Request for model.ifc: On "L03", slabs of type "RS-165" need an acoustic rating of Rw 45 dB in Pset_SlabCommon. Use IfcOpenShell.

First a look at what the model holds.

```python
import ifcopenshell
import ifcopenshell.util.element

model = ifcopenshell.open("model.ifc")
print(model.schema)
storey = next(s for s in model.by_type("IfcBuildingStorey") if s.Name == "L03")
slabs = [e for e in ifcopenshell.util.element.get_decomposition(storey) if e.is_a("IfcSlab")]
seen = {}
for e in slabs:
    element_type = ifcopenshell.util.element.get_type(e)
    key = (element_type.Name if element_type != e and element_type else None, ifcopenshell.util.element.get_pset(e, "Pset_SlabCommon", "AcousticRating"))
    seen[key] = seen.get(key, 0) + 1
for (name, value), count in sorted(seen.items(), key=str):
    print(count, "x", name, "|", value)
```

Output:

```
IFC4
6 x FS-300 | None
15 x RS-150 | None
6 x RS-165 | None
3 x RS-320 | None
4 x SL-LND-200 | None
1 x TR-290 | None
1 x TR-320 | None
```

```python
import ifcopenshell
import ifcopenshell.api.pset
import ifcopenshell.util.element

model = ifcopenshell.open("model.ifc")

storey = next(s for s in model.by_type("IfcBuildingStorey") if s.Name == "L03")
slabs = [e for e in ifcopenshell.util.element.get_decomposition(storey) if e.is_a("IfcSlab")]

count = 0
for e in slabs:
    element_type = ifcopenshell.util.element.get_type(e)
    if element_type in (None, e) or element_type.Name != "RS-165":
        continue
    # add_pset returns the element's existing set when there is one.
    pset = ifcopenshell.api.pset.add_pset(model, product=e, name="Pset_SlabCommon")
    ifcopenshell.api.pset.edit_pset(model, pset=pset, properties={"AcousticRating": "Rw 45 dB"})
    count += 1

print(count, "slabs updated")

model.write("model_rev.ifc")
```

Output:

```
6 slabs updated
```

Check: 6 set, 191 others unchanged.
